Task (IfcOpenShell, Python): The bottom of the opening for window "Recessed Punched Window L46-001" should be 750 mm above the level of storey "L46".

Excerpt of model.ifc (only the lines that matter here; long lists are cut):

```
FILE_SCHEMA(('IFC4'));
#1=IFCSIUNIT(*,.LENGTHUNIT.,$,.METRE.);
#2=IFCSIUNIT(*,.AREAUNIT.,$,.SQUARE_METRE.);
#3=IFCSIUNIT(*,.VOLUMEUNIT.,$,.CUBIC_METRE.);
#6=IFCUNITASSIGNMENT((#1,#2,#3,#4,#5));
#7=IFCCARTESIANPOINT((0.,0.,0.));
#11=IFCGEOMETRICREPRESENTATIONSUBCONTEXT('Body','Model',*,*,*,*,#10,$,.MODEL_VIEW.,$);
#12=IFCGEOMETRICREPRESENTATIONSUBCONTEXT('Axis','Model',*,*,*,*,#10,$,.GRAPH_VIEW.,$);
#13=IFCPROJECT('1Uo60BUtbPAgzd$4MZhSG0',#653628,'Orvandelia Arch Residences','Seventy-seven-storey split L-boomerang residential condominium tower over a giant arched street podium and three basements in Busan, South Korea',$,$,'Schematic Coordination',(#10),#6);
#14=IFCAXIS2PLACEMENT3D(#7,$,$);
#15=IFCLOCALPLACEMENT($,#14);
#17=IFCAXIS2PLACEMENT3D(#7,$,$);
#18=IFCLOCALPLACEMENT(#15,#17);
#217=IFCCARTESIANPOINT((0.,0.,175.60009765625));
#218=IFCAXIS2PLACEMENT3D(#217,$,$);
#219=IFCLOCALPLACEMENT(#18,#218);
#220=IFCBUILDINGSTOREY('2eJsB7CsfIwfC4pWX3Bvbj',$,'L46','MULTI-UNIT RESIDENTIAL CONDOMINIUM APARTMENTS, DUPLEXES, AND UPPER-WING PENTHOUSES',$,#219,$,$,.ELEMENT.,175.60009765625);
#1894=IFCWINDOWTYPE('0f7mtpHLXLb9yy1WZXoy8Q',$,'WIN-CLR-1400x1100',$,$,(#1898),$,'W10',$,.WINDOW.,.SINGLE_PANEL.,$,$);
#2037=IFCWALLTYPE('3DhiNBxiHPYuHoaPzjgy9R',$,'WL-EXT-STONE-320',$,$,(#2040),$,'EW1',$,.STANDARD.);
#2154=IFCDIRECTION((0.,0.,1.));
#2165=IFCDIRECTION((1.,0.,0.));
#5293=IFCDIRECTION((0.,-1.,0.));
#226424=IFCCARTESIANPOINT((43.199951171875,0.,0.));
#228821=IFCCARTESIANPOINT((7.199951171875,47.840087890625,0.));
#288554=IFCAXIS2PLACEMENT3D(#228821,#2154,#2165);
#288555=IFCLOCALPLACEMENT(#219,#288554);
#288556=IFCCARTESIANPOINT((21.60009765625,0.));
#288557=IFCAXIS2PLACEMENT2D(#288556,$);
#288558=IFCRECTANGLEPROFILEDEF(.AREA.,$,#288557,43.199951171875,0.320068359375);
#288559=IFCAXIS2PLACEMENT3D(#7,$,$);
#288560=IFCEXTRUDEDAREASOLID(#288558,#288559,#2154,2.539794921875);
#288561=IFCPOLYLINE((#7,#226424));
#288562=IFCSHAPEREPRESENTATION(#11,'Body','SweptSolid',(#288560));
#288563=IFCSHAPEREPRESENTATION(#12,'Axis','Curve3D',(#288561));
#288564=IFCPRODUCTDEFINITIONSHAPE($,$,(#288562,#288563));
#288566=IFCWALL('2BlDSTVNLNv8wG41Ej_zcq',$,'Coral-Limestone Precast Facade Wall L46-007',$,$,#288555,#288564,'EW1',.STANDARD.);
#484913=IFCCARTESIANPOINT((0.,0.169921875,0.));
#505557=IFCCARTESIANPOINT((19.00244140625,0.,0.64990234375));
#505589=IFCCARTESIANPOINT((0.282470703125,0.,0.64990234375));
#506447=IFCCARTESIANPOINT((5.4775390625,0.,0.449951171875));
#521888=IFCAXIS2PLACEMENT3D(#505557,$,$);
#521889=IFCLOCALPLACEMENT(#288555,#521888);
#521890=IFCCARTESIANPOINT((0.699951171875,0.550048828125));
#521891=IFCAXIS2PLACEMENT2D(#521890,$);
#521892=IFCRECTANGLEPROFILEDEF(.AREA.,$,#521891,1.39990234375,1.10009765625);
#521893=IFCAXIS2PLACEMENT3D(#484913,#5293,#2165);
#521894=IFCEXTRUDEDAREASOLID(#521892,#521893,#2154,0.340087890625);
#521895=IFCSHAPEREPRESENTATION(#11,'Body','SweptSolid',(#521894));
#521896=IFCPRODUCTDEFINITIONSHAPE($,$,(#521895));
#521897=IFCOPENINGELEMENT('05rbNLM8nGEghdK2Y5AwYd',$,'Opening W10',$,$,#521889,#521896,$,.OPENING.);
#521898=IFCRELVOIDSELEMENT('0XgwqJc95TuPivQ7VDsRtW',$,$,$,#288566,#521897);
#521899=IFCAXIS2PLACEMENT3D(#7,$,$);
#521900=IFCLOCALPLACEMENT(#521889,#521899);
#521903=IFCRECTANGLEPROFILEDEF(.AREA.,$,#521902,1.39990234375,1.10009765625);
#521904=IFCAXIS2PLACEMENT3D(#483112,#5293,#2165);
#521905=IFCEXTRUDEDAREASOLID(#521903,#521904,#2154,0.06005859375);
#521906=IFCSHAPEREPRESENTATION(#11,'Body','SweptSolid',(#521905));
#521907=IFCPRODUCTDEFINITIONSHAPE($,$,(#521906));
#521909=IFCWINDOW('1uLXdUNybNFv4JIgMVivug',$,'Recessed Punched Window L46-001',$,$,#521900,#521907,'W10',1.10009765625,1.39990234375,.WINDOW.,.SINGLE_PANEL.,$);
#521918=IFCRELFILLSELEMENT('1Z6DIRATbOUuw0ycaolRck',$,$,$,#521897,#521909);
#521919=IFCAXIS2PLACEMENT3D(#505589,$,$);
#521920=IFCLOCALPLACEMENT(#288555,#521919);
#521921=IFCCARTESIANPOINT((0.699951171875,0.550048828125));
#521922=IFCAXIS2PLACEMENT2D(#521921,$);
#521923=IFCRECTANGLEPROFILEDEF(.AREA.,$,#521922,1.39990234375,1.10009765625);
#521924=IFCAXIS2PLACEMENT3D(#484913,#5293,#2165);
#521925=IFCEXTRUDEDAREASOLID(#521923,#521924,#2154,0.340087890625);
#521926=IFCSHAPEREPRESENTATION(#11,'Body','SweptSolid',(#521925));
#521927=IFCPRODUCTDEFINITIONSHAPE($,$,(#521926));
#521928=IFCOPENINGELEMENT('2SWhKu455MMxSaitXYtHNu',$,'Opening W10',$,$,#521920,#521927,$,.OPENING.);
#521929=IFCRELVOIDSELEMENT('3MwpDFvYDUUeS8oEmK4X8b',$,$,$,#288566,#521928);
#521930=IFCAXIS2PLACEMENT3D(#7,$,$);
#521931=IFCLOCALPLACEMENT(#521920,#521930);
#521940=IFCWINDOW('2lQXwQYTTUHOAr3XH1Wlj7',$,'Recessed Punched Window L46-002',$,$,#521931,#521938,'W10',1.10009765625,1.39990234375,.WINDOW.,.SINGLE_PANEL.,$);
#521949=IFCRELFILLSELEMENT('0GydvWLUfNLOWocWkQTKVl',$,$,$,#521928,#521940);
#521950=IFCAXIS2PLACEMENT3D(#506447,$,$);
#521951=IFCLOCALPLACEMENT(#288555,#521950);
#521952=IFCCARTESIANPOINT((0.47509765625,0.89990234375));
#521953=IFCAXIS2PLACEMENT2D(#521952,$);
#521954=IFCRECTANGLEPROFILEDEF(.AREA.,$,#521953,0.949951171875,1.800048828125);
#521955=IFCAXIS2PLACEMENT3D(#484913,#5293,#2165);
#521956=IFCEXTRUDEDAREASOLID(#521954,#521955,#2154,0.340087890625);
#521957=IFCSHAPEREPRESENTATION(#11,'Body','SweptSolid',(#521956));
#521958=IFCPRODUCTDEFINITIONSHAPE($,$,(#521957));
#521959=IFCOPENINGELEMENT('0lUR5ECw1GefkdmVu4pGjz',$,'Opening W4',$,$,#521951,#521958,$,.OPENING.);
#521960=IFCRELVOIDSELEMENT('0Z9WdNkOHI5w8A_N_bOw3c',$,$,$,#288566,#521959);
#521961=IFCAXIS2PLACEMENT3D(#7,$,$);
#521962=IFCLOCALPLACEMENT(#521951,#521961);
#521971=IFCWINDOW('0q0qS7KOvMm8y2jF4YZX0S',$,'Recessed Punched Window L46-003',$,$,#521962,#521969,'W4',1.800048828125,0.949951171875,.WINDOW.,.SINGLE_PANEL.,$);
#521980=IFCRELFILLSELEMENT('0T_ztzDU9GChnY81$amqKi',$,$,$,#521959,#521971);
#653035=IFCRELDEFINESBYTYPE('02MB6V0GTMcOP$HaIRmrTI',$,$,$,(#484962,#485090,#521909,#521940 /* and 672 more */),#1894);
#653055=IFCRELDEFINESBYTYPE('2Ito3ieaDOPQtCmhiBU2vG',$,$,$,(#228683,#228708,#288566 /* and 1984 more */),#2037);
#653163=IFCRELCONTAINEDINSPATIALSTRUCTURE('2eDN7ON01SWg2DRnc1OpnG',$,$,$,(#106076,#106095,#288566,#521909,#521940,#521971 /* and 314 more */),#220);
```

```python
import numpy as np
import ifcopenshell
import ifcopenshell.api.geometry
import ifcopenshell.geom
import ifcopenshell.util.element
import ifcopenshell.util.placement
import ifcopenshell.util.shape
import ifcopenshell.util.unit

model = ifcopenshell.open("model.ifc")
unit_scale = ifcopenshell.util.unit.calculate_unit_scale(model)

window = model.by_guid("1uLXdUNybNFv4JIgMVivug")
opening = window.FillsVoids[0].RelatingOpeningElement
storey = ifcopenshell.util.element.get_container(window, ifc_class="IfcBuildingStorey")
level = ifcopenshell.util.placement.get_local_placement(storey.ObjectPlacement)[2, 3]

# The opening's origin need not be at the sill, so measure its lowest point.
shape = ifcopenshell.geom.create_shape(ifcopenshell.geom.settings(), opening)
bottom = ifcopenshell.util.shape.get_shape_bottom_elevation(shape, shape.geometry) / unit_scale
dz = level + 0.75 / unit_scale - bottom

shift = np.array([0.0, 0.0, dz])
# The window is placed relative to its opening, so it follows when the opening moves.
matrix = ifcopenshell.util.placement.get_local_placement(opening.ObjectPlacement)
matrix[:3, 3] += shift
ifcopenshell.api.geometry.edit_object_placement(
    model, product=opening, matrix=matrix, is_si=False, should_transform_children=True
)

print(f"moved by {dz * unit_scale:+.3f} m")

model.write("model-out.ifc")
```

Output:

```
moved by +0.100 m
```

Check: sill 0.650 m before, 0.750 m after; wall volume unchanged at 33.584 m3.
